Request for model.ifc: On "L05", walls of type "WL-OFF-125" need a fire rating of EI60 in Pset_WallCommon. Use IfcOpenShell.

First a look at what the model holds.

```python
import ifcopenshell
import ifcopenshell.util.element

model = ifcopenshell.open("model.ifc")
print(model.schema)
storey = next(s for s in model.by_type("IfcBuildingStorey") if s.Name == "L05")
walls = [e for e in ifcopenshell.util.element.get_decomposition(storey) if e.is_a("IfcWall")]
seen = {}
for e in walls:
    element_type = ifcopenshell.util.element.get_type(e)
    key = (element_type.Name if element_type != e and element_type else None, ifcopenshell.util.element.get_pset(e, "Pset_WallCommon", "FireRating"))
    seen[key] = seen.get(key, 0) + 1
for (name, value), count in sorted(seen.items(), key=str):
    print(count, "x", name, "|", value)
```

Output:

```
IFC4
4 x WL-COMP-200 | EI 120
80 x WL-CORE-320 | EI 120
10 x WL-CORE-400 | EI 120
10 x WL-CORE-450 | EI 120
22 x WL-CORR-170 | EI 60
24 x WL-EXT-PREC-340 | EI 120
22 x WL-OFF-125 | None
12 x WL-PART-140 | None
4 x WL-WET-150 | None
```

```python
import ifcopenshell
import ifcopenshell.api.pset
import ifcopenshell.util.element

model = ifcopenshell.open("model.ifc")

storey = next(s for s in model.by_type("IfcBuildingStorey") if s.Name == "L05")
walls = [e for e in ifcopenshell.util.element.get_decomposition(storey) if e.is_a("IfcWall")]

count = 0
for e in walls:
    element_type = ifcopenshell.util.element.get_type(e)
    if element_type in (None, e) or element_type.Name != "WL-OFF-125":
        continue
    # add_pset returns the element's existing set when there is one.
    pset = ifcopenshell.api.pset.add_pset(model, product=e, name="Pset_WallCommon")
    ifcopenshell.api.pset.edit_pset(model, pset=pset, properties={"FireRating": "EI60"})
    count += 1

print(count, "walls updated")

model.write("model_edited.ifc")
```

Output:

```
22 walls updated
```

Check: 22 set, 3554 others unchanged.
